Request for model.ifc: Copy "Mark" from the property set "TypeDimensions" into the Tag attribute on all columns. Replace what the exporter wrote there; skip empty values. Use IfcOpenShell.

First a look at what the model holds.

```python
import ifcopenshell
import ifcopenshell.util.element

model = ifcopenshell.open("model.ifc")
print(model.schema)
columns = model.by_type("IfcColumn")
print(len(columns), "columns")
for e in columns[:8]:
    source = ifcopenshell.util.element.get_pset(e, "TypeDimensions", "Mark")
    target = e.Tag
    print(e.id(), repr(source), repr(target), sep=" | ")
```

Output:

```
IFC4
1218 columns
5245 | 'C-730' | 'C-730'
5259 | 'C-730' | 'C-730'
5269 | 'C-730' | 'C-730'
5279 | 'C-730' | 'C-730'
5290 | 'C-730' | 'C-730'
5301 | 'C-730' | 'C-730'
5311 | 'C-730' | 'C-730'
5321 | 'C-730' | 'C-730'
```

```python
import ifcopenshell
import ifcopenshell.util.element

model = ifcopenshell.open("model.ifc")

count = 0
for e in model.by_type("IfcColumn"):
    value = ifcopenshell.util.element.get_pset(e, "TypeDimensions", "Mark")
    current = e.Tag
    if not value or not value.strip() or current == value:
        continue
    e.Tag = value
    count += 1

print(count, "columns updated")

model.write("model_rev.ifc")
```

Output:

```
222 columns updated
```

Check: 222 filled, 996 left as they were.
